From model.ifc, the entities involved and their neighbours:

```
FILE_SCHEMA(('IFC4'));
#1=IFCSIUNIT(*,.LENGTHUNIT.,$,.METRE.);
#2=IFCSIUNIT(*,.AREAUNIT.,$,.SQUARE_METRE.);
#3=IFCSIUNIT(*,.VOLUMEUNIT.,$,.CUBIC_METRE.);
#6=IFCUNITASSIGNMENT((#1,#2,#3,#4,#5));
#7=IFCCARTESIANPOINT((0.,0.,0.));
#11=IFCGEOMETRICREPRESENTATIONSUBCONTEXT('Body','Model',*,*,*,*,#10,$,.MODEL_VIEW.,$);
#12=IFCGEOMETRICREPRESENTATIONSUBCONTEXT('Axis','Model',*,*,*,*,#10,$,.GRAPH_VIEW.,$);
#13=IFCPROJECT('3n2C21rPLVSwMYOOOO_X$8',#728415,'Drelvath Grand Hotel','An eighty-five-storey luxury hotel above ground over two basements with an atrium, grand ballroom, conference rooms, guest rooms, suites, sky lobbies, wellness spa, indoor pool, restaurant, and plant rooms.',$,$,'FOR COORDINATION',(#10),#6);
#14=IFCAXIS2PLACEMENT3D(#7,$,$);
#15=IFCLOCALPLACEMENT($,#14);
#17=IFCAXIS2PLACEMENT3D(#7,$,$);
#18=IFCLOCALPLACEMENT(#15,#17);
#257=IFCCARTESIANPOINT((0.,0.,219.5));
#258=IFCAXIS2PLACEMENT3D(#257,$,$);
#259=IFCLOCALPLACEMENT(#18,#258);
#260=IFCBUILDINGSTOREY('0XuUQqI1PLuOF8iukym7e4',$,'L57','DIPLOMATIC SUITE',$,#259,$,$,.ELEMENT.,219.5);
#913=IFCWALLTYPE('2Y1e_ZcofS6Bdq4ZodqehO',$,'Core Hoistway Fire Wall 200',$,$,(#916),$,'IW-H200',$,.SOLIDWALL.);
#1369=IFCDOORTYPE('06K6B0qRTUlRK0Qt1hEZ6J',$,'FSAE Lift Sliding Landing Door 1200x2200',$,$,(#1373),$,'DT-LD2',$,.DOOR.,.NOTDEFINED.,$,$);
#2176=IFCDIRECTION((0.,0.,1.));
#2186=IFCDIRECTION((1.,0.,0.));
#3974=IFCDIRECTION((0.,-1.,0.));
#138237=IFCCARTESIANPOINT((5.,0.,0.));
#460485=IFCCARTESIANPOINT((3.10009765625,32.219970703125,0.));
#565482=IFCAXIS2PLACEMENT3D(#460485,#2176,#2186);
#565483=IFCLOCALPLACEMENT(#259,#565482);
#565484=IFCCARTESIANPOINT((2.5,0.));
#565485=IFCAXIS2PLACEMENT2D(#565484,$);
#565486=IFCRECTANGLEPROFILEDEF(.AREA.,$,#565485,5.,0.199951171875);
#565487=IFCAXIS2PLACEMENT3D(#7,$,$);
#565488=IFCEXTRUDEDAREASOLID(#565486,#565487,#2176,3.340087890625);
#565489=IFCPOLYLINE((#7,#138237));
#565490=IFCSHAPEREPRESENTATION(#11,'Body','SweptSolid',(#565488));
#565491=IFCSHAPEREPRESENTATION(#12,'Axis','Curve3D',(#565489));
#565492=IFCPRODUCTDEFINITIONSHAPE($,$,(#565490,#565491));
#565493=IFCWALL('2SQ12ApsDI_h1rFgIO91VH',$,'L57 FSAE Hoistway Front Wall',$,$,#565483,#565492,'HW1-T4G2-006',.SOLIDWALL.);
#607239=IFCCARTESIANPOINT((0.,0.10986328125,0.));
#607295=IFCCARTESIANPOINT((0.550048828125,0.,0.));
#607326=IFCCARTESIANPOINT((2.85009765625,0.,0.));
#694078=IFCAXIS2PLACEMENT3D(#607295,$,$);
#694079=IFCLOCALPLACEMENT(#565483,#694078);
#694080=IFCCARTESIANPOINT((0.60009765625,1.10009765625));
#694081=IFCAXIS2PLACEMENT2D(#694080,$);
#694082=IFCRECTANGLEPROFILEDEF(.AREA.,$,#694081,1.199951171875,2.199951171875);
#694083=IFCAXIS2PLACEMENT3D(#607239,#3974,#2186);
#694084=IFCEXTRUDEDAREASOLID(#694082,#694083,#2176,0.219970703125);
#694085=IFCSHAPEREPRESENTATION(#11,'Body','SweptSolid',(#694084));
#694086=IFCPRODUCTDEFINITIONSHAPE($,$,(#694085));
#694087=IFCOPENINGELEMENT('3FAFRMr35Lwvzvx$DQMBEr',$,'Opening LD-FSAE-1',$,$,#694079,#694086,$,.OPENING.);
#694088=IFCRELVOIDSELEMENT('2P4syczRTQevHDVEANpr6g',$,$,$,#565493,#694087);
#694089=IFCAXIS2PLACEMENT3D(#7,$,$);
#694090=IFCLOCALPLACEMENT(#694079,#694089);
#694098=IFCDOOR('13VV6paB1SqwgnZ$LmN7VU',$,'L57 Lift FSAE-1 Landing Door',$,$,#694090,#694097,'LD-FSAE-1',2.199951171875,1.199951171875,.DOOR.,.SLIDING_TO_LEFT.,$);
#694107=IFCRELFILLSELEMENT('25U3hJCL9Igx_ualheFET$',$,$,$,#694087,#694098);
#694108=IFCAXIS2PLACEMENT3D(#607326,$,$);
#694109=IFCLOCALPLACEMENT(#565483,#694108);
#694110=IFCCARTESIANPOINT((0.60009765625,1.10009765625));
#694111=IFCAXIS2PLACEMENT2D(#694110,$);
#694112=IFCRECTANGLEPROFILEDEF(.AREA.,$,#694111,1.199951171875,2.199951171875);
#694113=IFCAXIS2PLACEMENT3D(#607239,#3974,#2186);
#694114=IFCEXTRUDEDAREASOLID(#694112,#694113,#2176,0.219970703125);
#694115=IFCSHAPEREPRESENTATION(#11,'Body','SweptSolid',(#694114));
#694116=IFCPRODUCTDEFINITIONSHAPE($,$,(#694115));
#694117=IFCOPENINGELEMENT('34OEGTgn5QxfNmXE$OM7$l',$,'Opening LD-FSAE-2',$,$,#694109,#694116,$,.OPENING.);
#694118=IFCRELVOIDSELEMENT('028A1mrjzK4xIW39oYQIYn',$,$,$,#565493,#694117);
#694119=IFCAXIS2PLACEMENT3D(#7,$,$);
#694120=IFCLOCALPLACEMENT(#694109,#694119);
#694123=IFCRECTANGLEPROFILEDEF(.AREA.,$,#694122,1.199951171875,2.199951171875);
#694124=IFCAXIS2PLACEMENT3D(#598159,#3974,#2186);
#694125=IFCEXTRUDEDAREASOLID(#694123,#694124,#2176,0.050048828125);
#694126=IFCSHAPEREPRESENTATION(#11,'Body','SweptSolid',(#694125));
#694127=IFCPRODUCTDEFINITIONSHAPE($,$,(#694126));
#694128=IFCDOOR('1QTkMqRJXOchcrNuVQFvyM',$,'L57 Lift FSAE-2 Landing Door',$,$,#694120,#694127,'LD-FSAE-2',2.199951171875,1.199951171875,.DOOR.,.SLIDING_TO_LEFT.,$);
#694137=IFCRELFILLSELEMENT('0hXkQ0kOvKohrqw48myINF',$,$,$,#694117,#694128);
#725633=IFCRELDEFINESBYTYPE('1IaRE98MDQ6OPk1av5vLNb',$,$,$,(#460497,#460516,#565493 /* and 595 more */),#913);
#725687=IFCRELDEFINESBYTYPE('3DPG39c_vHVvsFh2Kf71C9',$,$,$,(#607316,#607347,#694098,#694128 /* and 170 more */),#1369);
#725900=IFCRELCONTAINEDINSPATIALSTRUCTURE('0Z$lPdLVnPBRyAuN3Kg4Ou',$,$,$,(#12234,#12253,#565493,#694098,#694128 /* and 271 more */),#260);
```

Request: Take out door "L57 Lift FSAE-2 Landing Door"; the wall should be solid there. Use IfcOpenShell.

```python
import ifcopenshell
import ifcopenshell.api.feature
import ifcopenshell.api.root
import ifcopenshell.geom
import ifcopenshell.util.shape

model = ifcopenshell.open("model.ifc")
settings = ifcopenshell.geom.settings()


def volume(element):
    """Net volume in cubic metres, openings subtracted."""
    shape = ifcopenshell.geom.create_shape(settings, element)
    return ifcopenshell.util.shape.get_volume(shape.geometry)


door = model.by_id(694128)
opening = door.FillsVoids[0].RelatingOpeningElement
wall = opening.VoidsElements[0].RelatingBuildingElement
before = volume(wall)

ifcopenshell.api.root.remove_product(model, product=door)
ifcopenshell.api.feature.remove_feature(model, feature=opening)

after = volume(wall)

print(f"wall volume {before:.3f} -> {after:.3f} m3")

model.write("model_rev.ifc")
```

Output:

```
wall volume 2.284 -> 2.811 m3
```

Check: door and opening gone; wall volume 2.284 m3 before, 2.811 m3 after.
